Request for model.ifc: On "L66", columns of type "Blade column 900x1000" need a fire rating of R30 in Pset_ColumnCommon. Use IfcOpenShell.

First a look at what the model holds.

```python
import ifcopenshell
import ifcopenshell.util.element

model = ifcopenshell.open("model.ifc")
print(model.schema)
storey = next(s for s in model.by_type("IfcBuildingStorey") if s.Name == "L66")
columns = [e for e in ifcopenshell.util.element.get_decomposition(storey) if e.is_a("IfcColumn")]
seen = {}
for e in columns:
    element_type = ifcopenshell.util.element.get_type(e)
    key = (element_type.Name if element_type != e and element_type else None, ifcopenshell.util.element.get_pset(e, "Pset_ColumnCommon", "FireRating"))
    seen[key] = seen.get(key, 0) + 1
for (name, value), count in sorted(seen.items(), key=str):
    print(count, "x", name, "|", value)
```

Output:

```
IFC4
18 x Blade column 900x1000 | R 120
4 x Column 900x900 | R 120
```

```python
import ifcopenshell
import ifcopenshell.api.pset
import ifcopenshell.util.element

model = ifcopenshell.open("model.ifc")

storey = next(s for s in model.by_type("IfcBuildingStorey") if s.Name == "L66")
columns = [e for e in ifcopenshell.util.element.get_decomposition(storey) if e.is_a("IfcColumn")]

count = 0
for e in columns:
    element_type = ifcopenshell.util.element.get_type(e)
    if element_type in (None, e) or element_type.Name != "Blade column 900x1000":
        continue
    found = ifcopenshell.util.element.get_pset(e, "Pset_ColumnCommon", should_inherit=False)
    if found:
        pset = model.by_id(found["id"])
        if len(ifcopenshell.util.element.get_elements_by_pset(pset)) > 1:
            pset = ifcopenshell.api.pset.unshare_pset(model, products=[e], pset=pset)[0]
    else:
        pset = ifcopenshell.api.pset.add_pset(model, product=e, name="Pset_ColumnCommon")
    ifcopenshell.api.pset.edit_pset(model, pset=pset, properties={"FireRating": "R30"})
    count += 1

print(count, "columns updated")

model.write("model_edited.ifc")
```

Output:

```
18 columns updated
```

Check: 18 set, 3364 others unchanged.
